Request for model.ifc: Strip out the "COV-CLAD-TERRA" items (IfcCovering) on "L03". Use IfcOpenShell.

First a look at what the model holds.

```python
import ifcopenshell
import ifcopenshell.util.element

model = ifcopenshell.open("model.ifc")
print(model.schema)
storey = next(s for s in model.by_type("IfcBuildingStorey") if s.Name == "L03")
coverings = [e for e in ifcopenshell.util.element.get_decomposition(storey) if e.is_a("IfcCovering")]
seen = {}
for e in coverings:
    element_type = ifcopenshell.util.element.get_type(e)
    name = element_type.Name if element_type not in (None, e) else None
    seen[name] = seen.get(name, 0) + 1
for name, count in sorted(seen.items(), key=str):
    print(count, "x", name)
```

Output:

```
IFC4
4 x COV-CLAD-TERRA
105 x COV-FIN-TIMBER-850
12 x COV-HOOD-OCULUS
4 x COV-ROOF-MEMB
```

```python
import ifcopenshell
import ifcopenshell.api.root
import ifcopenshell.util.element

model = ifcopenshell.open("model.ifc")

storey = next(s for s in model.by_type("IfcBuildingStorey") if s.Name == "L03")
coverings = [e for e in ifcopenshell.util.element.get_decomposition(storey) if e.is_a("IfcCovering")]
targets = [e for e in coverings if (t := ifcopenshell.util.element.get_type(e)) not in (None, e) and t.Name == "COV-CLAD-TERRA"]

for e in targets:
    ifcopenshell.api.root.remove_product(model, product=e)
print(len(targets), "removed")

model.write("model_rev.ifc")
```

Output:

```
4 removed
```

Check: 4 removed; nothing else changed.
